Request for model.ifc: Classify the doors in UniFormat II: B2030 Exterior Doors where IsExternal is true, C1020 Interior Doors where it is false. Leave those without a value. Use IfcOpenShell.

First a look at what the model holds.

```python
import ifcopenshell
import ifcopenshell.util.element

model = ifcopenshell.open("model.ifc")
print(model.schema)
print("classifications:", [c.Name for c in model.by_type("IfcClassification")])
values = [ifcopenshell.util.element.get_pset(e, "Pset_DoorCommon", "IsExternal") for e in model.by_type("IfcDoor")]
for value in (True, False, None):
    print("IsExternal", value, values.count(value))
```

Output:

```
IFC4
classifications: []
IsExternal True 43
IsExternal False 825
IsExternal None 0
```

```python
import ifcopenshell
import ifcopenshell.api.classification
import ifcopenshell.util.element

model = ifcopenshell.open("model.ifc")

system = ifcopenshell.api.classification.add_classification(model, classification="UniFormat II")

doors = model.by_type("IfcDoor")
external = {e: ifcopenshell.util.element.get_pset(e, "Pset_DoorCommon", "IsExternal") for e in doors}
for flag, code, name in ((True, "B2030", "Exterior Doors"), (False, "C1020", "Interior Doors")):
    products = [e for e in doors if external[e] is flag]
    ifcopenshell.api.classification.add_reference(
        model, products=products, classification=system, identification=code, name=name
    )
    print(code, len(products))

model.write("model-out.ifc")
```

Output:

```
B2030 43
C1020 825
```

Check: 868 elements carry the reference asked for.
